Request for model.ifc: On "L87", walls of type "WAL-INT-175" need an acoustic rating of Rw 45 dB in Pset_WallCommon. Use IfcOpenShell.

First a look at what the model holds.

```python
import ifcopenshell
import ifcopenshell.util.element

model = ifcopenshell.open("model.ifc")
print(model.schema)
storey = next(s for s in model.by_type("IfcBuildingStorey") if s.Name == "L87")
walls = [e for e in ifcopenshell.util.element.get_decomposition(storey) if e.is_a("IfcWall")]
seen = {}
for e in walls:
    element_type = ifcopenshell.util.element.get_type(e)
    key = (element_type.Name if element_type != e and element_type else None, ifcopenshell.util.element.get_pset(e, "Pset_WallCommon", "AcousticRating"))
    seen[key] = seen.get(key, 0) + 1
for (name, value), count in sorted(seen.items(), key=str):
    print(count, "x", name, "|", value)
```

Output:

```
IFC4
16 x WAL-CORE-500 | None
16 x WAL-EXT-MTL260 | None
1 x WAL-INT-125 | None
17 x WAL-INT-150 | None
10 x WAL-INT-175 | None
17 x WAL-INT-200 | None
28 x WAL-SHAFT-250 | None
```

```python
import ifcopenshell
import ifcopenshell.api.pset
import ifcopenshell.util.element

model = ifcopenshell.open("model.ifc")

storey = next(s for s in model.by_type("IfcBuildingStorey") if s.Name == "L87")
walls = [e for e in ifcopenshell.util.element.get_decomposition(storey) if e.is_a("IfcWall")]

count = 0
for e in walls:
    element_type = ifcopenshell.util.element.get_type(e)
    if element_type in (None, e) or element_type.Name != "WAL-INT-175":
        continue
    found = ifcopenshell.util.element.get_pset(e, "Pset_WallCommon", should_inherit=False)
    if found:
        pset = model.by_id(found["id"])
        if len(ifcopenshell.util.element.get_elements_by_pset(pset)) > 1:
            pset = ifcopenshell.api.pset.unshare_pset(model, products=[e], pset=pset)[0]
    else:
        pset = ifcopenshell.api.pset.add_pset(model, product=e, name="Pset_WallCommon")
    ifcopenshell.api.pset.edit_pset(model, pset=pset, properties={"AcousticRating": "Rw 45 dB"})
    count += 1

print(count, "walls updated")

model.write("model-out.ifc")
```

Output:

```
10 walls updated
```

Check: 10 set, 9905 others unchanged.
